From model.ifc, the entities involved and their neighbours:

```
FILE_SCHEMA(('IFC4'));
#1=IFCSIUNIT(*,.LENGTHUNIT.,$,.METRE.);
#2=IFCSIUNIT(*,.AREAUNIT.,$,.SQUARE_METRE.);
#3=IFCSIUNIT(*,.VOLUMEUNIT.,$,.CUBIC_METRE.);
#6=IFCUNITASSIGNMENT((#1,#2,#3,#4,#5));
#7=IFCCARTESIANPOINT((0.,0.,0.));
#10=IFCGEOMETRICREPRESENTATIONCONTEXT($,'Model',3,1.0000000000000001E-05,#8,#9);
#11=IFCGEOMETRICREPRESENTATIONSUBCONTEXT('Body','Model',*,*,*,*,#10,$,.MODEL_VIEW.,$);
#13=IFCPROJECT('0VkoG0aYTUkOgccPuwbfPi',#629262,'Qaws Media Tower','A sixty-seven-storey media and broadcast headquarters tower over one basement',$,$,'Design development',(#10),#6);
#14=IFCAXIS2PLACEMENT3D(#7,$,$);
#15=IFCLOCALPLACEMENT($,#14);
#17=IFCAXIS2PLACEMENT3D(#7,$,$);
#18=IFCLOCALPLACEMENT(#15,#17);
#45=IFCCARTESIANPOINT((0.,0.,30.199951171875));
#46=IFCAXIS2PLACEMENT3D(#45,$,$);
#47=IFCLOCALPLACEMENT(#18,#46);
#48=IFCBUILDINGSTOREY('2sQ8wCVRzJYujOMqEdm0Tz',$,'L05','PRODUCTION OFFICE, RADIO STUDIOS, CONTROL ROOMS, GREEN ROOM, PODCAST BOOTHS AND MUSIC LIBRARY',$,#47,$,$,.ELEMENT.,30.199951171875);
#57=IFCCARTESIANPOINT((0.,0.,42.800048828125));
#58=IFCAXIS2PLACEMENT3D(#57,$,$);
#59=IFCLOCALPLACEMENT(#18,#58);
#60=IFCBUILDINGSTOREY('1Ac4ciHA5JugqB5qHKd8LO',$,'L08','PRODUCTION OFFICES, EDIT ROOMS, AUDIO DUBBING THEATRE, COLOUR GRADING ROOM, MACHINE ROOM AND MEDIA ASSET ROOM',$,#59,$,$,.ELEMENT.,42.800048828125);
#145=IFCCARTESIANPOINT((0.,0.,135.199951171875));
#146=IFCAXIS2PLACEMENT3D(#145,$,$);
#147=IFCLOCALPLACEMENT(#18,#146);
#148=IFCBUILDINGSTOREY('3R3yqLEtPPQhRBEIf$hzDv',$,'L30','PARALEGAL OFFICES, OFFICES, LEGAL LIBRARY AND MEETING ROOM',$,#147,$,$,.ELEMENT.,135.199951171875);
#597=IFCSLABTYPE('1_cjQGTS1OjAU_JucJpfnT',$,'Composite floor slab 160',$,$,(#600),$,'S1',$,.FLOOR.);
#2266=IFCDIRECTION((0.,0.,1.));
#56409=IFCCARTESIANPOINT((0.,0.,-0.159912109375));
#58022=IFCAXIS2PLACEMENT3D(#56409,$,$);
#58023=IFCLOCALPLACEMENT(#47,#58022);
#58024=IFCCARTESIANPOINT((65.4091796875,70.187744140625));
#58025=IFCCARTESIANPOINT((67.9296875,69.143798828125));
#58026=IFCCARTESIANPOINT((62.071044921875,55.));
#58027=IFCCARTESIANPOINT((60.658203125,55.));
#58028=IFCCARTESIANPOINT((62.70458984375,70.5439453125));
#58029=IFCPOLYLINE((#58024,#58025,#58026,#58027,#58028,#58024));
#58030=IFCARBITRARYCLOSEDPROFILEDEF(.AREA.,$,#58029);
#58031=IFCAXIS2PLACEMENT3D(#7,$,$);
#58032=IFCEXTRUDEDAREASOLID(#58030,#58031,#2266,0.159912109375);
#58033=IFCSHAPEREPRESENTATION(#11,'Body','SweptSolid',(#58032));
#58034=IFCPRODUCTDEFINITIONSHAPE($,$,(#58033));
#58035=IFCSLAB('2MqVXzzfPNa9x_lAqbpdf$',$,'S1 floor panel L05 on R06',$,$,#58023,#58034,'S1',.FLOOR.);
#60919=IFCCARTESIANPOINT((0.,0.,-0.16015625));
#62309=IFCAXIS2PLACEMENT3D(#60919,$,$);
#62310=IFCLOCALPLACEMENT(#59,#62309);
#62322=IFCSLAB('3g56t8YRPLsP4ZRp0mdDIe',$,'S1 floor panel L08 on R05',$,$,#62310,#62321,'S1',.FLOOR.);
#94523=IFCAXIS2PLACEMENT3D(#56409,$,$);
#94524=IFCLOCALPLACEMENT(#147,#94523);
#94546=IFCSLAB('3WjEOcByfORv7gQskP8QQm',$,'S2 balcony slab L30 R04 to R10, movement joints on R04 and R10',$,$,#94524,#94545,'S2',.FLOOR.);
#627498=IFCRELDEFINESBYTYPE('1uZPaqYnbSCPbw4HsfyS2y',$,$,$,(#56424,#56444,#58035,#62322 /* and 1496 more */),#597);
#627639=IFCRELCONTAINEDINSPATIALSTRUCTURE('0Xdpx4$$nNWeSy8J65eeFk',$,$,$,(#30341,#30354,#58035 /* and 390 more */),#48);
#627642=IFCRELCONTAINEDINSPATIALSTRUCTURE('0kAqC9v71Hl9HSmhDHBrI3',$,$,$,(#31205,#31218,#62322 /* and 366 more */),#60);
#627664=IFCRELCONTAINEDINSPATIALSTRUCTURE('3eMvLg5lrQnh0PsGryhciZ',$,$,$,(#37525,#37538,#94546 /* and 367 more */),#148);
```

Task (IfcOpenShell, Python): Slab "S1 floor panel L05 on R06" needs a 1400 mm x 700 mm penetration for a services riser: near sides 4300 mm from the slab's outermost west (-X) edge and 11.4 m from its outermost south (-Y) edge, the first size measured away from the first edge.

```python
import numpy as np
import ifcopenshell
import ifcopenshell.api.feature
import ifcopenshell.api.geometry
import ifcopenshell.api.root
import ifcopenshell.geom
import ifcopenshell.util.placement
import ifcopenshell.util.representation
import ifcopenshell.util.shape
import ifcopenshell.util.unit

model = ifcopenshell.open("model.ifc")
unit_scale = ifcopenshell.util.unit.calculate_unit_scale(model)
settings = ifcopenshell.geom.settings()


def volume(element):
    """Net volume in cubic metres, openings subtracted."""
    shape = ifcopenshell.geom.create_shape(settings, element)
    return ifcopenshell.util.shape.get_volume(shape.geometry)


slab = model.by_guid("2MqVXzzfPNa9x_lAqbpdf$")
before = volume(slab)

# Extent in the slab's own axes, in metres. The edges named are its -X and -Y sides.
slab_shape = ifcopenshell.geom.create_shape(settings, slab)
vertices = ifcopenshell.util.shape.get_vertices(slab_shape.geometry)
x_min, y_min, bottom = vertices.min(axis=0)
top = vertices[:, 2].max()

opening = ifcopenshell.api.root.create_entity(model, ifc_class="IfcOpeningElement", name="Services riser opening", predefined_type="OPENING")
context = ifcopenshell.util.representation.get_context(model, "Model", "Body", "MODEL_VIEW")
width, depth = 1.4, 0.7
outline = [(0.0, 0.0), (width, 0.0), (width, depth), (0.0, depth), (0.0, 0.0)]
# Overshoot both faces by 50 mm so the cut is clean.
shape = ifcopenshell.api.geometry.add_slab_representation(
    model, context=context, depth=top - bottom + 0.1, polyline=outline
)
ifcopenshell.api.geometry.assign_representation(model, product=opening, representation=shape)

matrix = ifcopenshell.util.placement.get_local_placement(slab.ObjectPlacement)
matrix[:, 3] = matrix @ np.append(np.array([x_min + 4.3, y_min + 11.4, bottom - 0.05]) / unit_scale, 1.0)
ifcopenshell.api.geometry.edit_object_placement(model, product=opening, matrix=matrix, is_si=False)
ifcopenshell.api.feature.add_feature(model, feature=opening, element=slab)

after = volume(slab)

print(f"slab volume {before:.3f} -> {after:.3f} m3")

model.write("model_v2.ifc")
```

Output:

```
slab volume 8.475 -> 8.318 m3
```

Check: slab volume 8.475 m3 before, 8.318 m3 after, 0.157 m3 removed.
